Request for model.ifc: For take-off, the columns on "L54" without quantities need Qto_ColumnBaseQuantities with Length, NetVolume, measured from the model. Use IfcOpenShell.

First a look at what the model holds.

```python
import ifcopenshell
import ifcopenshell.util.element
import ifcopenshell.util.unit

model = ifcopenshell.open("model.ifc")
print(model.schema)
for unit_type in ("LENGTHUNIT", "AREAUNIT", "VOLUMEUNIT"):
    print(unit_type, ifcopenshell.util.unit.calculate_unit_scale(model, unit_type))
storey = next(s for s in model.by_type("IfcBuildingStorey") if s.Name == "L54")
columns = [e for e in ifcopenshell.util.element.get_decomposition(storey) if e.is_a("IfcColumn")]
for e in sorted(columns, key=lambda e: e.id()):
    print(e.id(), e.is_a(), e.Name, list(ifcopenshell.util.element.get_psets(e, qtos_only=True)), sep=" | ")
```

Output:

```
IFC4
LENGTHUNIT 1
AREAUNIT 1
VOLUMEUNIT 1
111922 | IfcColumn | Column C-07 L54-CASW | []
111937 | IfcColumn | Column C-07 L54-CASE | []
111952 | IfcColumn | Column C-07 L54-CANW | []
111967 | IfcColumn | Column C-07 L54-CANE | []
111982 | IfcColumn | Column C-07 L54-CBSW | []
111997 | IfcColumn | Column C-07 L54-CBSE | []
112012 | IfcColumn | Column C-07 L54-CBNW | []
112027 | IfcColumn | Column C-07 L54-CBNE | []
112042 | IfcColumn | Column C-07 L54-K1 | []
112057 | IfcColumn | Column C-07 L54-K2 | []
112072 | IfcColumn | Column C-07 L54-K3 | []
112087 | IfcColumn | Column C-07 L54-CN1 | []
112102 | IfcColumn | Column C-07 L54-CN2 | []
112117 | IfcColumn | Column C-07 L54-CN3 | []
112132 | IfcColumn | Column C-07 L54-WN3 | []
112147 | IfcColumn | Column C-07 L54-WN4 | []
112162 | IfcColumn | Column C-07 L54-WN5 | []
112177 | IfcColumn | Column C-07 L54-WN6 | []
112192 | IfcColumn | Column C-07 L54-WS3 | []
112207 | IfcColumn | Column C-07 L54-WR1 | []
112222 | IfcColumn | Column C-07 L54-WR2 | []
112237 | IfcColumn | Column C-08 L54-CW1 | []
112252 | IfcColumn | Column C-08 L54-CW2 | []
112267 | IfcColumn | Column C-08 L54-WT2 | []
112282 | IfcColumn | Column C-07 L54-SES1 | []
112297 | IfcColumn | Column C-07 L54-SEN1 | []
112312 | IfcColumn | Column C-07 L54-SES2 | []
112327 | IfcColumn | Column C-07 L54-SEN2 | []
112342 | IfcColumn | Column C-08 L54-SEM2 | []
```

```python
import ifcopenshell
import ifcopenshell.api.pset
import ifcopenshell.geom
import ifcopenshell.util.element
import ifcopenshell.util.shape
import ifcopenshell.util.unit

model = ifcopenshell.open("model.ifc")
unit_scale = ifcopenshell.util.unit.calculate_unit_scale(model)
volume_scale = ifcopenshell.util.unit.calculate_unit_scale(model, "VOLUMEUNIT")
settings = ifcopenshell.geom.settings()

storey = next(s for s in model.by_type("IfcBuildingStorey") if s.Name == "L54")
columns = [e for e in ifcopenshell.util.element.get_decomposition(storey) if e.is_a("IfcColumn")]

for e in sorted(columns, key=lambda e: e.id()):
    if ifcopenshell.util.element.get_psets(e, qtos_only=True, should_inherit=False):
        continue
    # Geometry comes back in metres, in the element's own axes.
    shape = ifcopenshell.geom.create_shape(settings, e)
    values = {
        "Length": ifcopenshell.util.shape.get_z(shape.geometry) / unit_scale,
        "NetVolume": ifcopenshell.util.shape.get_volume(shape.geometry) / volume_scale,
    }
    qto = ifcopenshell.api.pset.add_qto(model, product=e, name="Qto_ColumnBaseQuantities")
    ifcopenshell.api.pset.edit_qto(model, qto=qto, properties=values)
    print(e.id(), {k: round(v, 3) for k, v in values.items()})

model.write("model-out.ifc")
```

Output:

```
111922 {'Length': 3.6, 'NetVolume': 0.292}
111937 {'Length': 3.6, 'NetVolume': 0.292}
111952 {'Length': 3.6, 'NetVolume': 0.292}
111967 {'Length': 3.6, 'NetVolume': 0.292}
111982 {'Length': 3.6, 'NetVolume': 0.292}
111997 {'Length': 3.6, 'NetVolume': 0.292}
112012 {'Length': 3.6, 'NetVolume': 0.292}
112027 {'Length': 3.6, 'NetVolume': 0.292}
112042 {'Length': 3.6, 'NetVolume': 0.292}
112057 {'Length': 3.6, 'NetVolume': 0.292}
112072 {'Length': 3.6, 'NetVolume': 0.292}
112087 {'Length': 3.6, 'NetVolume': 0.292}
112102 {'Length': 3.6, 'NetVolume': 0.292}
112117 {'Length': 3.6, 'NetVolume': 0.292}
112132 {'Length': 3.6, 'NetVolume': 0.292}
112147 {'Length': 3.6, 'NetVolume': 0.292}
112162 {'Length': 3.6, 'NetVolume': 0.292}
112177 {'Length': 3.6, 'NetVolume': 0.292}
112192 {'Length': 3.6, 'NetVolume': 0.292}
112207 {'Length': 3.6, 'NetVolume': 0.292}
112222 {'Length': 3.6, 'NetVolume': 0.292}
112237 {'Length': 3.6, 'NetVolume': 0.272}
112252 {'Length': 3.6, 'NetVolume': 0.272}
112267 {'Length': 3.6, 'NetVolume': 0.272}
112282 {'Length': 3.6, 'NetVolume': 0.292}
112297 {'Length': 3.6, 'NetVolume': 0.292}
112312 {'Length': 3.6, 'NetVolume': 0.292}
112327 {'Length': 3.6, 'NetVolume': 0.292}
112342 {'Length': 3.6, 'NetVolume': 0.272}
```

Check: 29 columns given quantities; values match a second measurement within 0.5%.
